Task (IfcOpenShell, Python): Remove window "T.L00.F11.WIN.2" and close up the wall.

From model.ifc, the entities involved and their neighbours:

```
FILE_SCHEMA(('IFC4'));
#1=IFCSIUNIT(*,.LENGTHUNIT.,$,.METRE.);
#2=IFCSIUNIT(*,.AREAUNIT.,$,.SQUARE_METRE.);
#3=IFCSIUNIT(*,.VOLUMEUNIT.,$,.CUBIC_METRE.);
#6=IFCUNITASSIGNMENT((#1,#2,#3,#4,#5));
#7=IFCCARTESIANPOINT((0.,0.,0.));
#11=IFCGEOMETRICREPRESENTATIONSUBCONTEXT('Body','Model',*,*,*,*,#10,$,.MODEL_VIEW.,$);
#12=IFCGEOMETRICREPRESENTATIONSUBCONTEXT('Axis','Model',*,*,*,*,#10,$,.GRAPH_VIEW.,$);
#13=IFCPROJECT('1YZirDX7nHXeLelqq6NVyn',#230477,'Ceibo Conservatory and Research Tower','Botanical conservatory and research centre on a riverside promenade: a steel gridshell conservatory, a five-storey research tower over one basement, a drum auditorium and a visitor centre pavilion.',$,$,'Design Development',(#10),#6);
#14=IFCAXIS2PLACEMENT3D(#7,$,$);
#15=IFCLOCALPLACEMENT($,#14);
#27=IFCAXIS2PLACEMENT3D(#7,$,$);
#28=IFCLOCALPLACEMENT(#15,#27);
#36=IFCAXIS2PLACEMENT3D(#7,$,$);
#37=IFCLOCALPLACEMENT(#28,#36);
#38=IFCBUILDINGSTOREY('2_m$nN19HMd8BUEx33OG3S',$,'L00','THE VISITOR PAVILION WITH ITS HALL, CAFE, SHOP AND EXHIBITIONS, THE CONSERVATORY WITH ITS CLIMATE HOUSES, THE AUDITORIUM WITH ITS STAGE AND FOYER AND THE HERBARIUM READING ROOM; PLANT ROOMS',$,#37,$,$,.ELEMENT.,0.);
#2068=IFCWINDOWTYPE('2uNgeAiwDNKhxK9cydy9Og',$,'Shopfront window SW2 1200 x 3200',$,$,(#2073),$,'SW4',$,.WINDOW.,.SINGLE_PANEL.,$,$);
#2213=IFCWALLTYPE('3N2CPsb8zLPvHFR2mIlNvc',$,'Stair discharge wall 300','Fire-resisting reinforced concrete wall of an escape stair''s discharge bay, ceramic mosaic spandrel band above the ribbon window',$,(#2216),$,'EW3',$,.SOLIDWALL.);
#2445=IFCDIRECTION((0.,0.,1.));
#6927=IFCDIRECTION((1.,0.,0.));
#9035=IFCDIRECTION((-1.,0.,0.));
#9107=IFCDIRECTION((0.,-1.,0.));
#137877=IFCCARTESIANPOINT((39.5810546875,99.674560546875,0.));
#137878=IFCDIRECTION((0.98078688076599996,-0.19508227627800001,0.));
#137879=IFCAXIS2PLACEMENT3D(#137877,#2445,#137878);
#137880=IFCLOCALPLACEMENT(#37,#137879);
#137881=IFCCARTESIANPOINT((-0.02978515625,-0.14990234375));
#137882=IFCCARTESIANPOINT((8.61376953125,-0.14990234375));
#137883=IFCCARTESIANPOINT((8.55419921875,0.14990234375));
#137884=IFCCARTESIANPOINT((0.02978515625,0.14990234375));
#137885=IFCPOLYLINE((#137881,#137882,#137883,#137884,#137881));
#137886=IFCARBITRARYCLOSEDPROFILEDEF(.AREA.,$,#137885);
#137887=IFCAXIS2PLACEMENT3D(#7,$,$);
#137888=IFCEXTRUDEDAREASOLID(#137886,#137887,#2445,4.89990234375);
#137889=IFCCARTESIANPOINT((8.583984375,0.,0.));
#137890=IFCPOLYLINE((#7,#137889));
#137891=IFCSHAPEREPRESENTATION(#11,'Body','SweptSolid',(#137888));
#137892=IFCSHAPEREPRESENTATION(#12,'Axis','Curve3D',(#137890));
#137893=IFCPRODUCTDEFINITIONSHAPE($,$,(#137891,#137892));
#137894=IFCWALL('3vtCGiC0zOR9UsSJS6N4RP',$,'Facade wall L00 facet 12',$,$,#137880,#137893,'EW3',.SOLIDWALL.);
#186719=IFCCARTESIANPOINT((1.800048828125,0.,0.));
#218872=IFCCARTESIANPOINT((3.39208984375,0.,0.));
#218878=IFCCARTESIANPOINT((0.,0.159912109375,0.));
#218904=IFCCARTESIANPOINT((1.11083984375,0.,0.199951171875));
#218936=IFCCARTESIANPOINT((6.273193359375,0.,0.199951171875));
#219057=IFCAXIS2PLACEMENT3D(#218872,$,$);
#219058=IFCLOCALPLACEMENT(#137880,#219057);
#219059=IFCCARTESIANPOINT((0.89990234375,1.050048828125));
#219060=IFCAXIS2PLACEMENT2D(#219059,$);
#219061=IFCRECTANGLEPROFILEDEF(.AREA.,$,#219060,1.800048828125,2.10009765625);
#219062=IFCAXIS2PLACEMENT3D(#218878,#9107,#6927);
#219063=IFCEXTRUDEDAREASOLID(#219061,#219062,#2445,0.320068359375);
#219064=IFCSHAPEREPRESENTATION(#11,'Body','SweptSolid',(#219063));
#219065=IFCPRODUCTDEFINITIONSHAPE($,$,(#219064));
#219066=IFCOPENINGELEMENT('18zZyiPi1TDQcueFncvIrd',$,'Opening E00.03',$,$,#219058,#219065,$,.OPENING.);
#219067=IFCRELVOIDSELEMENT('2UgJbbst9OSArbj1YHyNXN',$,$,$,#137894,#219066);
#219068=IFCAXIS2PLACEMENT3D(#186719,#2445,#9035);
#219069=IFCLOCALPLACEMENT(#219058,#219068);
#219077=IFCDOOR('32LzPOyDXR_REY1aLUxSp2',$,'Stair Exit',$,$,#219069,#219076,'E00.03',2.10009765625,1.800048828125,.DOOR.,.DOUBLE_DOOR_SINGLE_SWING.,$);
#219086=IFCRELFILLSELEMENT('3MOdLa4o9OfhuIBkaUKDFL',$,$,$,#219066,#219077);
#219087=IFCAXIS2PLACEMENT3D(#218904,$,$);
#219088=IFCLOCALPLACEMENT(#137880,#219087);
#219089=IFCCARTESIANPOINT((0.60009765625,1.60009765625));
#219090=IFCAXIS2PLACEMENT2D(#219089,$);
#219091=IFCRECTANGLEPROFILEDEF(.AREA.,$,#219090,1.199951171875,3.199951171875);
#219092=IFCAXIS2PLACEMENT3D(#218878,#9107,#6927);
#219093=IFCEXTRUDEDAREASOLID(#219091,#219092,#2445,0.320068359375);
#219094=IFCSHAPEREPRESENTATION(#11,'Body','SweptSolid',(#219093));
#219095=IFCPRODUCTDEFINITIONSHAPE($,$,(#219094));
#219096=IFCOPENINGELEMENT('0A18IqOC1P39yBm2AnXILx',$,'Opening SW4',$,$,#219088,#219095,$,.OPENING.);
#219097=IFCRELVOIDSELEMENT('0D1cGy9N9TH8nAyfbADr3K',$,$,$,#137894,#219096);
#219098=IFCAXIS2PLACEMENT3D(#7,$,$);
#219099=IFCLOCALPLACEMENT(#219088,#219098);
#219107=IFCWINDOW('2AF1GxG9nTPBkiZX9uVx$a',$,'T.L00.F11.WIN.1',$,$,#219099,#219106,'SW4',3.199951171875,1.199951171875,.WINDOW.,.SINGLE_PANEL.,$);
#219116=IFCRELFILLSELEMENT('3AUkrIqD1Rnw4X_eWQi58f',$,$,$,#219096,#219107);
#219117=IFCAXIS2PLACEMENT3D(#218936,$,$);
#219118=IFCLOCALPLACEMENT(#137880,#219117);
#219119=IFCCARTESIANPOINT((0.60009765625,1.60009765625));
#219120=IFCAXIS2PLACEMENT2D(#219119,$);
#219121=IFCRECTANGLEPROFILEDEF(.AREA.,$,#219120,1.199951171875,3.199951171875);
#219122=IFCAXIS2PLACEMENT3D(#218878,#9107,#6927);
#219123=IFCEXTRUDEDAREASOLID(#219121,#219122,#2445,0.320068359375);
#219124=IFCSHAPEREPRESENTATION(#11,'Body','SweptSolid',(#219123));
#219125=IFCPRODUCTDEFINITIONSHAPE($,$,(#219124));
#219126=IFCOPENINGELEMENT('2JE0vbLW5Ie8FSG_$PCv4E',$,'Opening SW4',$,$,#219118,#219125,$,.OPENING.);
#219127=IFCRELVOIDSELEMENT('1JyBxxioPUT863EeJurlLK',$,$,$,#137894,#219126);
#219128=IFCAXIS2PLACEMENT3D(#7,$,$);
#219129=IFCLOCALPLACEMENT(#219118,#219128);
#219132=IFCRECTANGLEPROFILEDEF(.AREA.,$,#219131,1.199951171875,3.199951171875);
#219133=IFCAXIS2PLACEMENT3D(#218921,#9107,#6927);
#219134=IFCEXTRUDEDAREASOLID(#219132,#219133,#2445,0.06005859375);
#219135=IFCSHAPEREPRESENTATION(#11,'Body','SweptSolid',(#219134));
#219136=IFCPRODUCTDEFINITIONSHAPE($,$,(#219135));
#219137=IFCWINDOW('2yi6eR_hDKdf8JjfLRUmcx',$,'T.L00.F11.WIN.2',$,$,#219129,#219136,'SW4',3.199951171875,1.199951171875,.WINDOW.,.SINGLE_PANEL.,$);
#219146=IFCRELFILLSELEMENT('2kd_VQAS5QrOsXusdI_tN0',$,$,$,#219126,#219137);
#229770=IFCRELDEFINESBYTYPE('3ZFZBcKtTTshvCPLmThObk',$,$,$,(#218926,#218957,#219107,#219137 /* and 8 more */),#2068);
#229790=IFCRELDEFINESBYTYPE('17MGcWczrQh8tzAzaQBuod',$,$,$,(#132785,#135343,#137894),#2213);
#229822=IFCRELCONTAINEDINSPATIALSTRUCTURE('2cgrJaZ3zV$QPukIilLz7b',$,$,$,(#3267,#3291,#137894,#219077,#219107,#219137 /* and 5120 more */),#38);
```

```python
import ifcopenshell
import ifcopenshell.api.feature
import ifcopenshell.api.root
import ifcopenshell.geom
import ifcopenshell.util.shape

model = ifcopenshell.open("model.ifc")
settings = ifcopenshell.geom.settings()


def volume(element):
    """Net volume in cubic metres, openings subtracted."""
    shape = ifcopenshell.geom.create_shape(settings, element)
    return ifcopenshell.util.shape.get_volume(shape.geometry)


window = model.by_guid("2yi6eR_hDKdf8JjfLRUmcx")
opening = window.FillsVoids[0].RelatingOpeningElement
wall = opening.VoidsElements[0].RelatingBuildingElement
before = volume(wall)

ifcopenshell.api.root.remove_product(model, product=window)
ifcopenshell.api.feature.remove_feature(model, feature=opening)

after = volume(wall)

print(f"wall volume {before:.3f} -> {after:.3f} m3")

model.write("model_rev.ifc")
```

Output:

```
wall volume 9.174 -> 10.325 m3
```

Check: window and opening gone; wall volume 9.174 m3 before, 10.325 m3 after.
